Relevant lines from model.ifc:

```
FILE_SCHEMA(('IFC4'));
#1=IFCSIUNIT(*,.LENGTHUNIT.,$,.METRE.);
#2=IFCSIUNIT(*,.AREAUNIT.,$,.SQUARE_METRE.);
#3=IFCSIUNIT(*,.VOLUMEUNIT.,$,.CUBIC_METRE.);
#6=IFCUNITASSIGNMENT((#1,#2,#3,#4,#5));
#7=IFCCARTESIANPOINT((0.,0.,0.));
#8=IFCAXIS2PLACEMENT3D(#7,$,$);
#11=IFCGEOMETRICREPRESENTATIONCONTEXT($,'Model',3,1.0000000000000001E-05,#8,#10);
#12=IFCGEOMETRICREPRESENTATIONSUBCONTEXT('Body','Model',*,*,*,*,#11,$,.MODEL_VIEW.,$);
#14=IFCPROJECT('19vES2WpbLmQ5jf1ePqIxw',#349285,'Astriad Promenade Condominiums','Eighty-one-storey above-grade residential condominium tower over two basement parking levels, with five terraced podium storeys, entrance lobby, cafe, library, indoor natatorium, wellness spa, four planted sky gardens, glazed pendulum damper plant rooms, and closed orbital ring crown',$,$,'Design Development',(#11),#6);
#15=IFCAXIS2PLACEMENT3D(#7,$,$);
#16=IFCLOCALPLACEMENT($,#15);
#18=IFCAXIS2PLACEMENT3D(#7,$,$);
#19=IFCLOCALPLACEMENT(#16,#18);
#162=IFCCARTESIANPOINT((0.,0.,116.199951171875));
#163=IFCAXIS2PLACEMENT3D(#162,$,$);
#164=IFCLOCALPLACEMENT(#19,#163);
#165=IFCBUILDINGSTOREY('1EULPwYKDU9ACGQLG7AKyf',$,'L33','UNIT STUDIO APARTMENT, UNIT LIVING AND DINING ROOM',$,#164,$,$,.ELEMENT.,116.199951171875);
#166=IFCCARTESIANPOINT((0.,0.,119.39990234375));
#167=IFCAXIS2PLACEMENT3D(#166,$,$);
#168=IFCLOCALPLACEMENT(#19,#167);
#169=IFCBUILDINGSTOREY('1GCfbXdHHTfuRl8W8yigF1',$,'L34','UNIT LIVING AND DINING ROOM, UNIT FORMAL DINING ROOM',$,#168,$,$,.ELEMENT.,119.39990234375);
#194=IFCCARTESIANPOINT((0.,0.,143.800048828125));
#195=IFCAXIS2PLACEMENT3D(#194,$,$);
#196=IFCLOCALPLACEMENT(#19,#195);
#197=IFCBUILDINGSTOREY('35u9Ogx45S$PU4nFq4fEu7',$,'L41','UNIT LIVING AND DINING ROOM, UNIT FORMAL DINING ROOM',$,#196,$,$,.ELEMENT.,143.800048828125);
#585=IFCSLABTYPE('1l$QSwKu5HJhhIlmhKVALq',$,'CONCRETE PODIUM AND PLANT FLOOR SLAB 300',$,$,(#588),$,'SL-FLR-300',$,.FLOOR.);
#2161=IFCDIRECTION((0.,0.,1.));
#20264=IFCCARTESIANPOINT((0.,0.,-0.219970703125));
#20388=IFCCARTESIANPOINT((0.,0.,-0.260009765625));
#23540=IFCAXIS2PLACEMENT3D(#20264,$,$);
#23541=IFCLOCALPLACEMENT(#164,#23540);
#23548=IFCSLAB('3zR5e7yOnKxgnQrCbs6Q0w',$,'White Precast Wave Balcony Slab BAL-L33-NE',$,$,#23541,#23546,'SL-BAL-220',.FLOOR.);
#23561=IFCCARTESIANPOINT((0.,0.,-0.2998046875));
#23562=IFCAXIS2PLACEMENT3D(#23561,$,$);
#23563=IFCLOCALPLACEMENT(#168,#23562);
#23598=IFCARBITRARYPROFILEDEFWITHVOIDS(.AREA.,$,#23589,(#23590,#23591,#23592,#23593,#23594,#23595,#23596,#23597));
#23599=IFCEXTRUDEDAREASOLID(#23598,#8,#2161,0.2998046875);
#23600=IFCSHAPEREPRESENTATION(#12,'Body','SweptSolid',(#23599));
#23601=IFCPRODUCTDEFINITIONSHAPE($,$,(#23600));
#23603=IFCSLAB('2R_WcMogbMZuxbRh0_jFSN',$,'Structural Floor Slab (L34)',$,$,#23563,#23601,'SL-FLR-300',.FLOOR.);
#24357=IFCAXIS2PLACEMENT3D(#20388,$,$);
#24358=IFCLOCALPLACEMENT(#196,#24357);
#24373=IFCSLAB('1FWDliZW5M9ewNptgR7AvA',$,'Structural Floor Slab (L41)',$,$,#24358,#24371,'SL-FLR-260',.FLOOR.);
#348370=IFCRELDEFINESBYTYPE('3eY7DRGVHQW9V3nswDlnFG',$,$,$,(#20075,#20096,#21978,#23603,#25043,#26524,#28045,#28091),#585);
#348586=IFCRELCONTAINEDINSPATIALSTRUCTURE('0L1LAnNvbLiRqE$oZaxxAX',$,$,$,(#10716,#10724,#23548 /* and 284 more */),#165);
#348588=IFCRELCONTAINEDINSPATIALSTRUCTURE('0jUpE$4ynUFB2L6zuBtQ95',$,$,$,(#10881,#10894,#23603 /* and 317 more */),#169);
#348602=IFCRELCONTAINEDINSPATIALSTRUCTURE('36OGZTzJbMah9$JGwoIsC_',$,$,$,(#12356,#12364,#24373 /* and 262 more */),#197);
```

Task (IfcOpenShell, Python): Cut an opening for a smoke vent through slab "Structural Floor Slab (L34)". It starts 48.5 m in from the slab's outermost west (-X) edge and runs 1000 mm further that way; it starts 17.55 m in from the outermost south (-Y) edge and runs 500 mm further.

```python
import numpy as np
import ifcopenshell
import ifcopenshell.api.feature
import ifcopenshell.api.geometry
import ifcopenshell.api.root
import ifcopenshell.geom
import ifcopenshell.util.placement
import ifcopenshell.util.representation
import ifcopenshell.util.shape
import ifcopenshell.util.unit

model = ifcopenshell.open("model.ifc")
unit_scale = ifcopenshell.util.unit.calculate_unit_scale(model)
settings = ifcopenshell.geom.settings()


def volume(element):
    """Net volume in cubic metres, openings subtracted."""
    shape = ifcopenshell.geom.create_shape(settings, element)
    return ifcopenshell.util.shape.get_volume(shape.geometry)


slab = model.by_guid("2R_WcMogbMZuxbRh0_jFSN")
before = volume(slab)

# Extent in the slab's own axes, in metres. The edges named are its -X and -Y sides.
slab_shape = ifcopenshell.geom.create_shape(settings, slab)
vertices = ifcopenshell.util.shape.get_vertices(slab_shape.geometry)
x_min, y_min, bottom = vertices.min(axis=0)
top = vertices[:, 2].max()

opening = ifcopenshell.api.root.create_entity(model, ifc_class="IfcOpeningElement", name="Smoke vent opening", predefined_type="OPENING")
context = ifcopenshell.util.representation.get_context(model, "Model", "Body", "MODEL_VIEW")
width, depth = 1, 0.5
outline = [(0.0, 0.0), (width, 0.0), (width, depth), (0.0, depth), (0.0, 0.0)]
# Overshoot both faces by 50 mm so the cut is clean.
shape = ifcopenshell.api.geometry.add_slab_representation(
    model, context=context, depth=top - bottom + 0.1, polyline=outline
)
ifcopenshell.api.geometry.assign_representation(model, product=opening, representation=shape)

matrix = ifcopenshell.util.placement.get_local_placement(slab.ObjectPlacement)
matrix[:, 3] = matrix @ np.append(np.array([x_min + 48.5, y_min + 17.55, bottom - 0.05]) / unit_scale, 1.0)
ifcopenshell.api.geometry.edit_object_placement(model, product=opening, matrix=matrix, is_si=False)
ifcopenshell.api.feature.add_feature(model, feature=opening, element=slab)

after = volume(slab)

print(f"slab volume {before:.3f} -> {after:.3f} m3")

model.write("model_v2.ifc")
```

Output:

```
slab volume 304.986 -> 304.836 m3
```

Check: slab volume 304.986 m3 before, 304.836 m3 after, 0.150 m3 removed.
